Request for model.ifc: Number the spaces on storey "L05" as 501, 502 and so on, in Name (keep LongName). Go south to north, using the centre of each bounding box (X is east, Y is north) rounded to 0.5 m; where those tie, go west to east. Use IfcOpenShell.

First a look at what the model holds.

```python
import ifcopenshell
import ifcopenshell.util.element
import ifcopenshell.util.placement

model = ifcopenshell.open("model.ifc")
print(model.schema)
storey = next(s for s in model.by_type("IfcBuildingStorey") if s.Name == "L05")
spaces = [e for e in ifcopenshell.util.element.get_decomposition(storey) if e.is_a("IfcSpace")]
for e in sorted(spaces, key=lambda e: e.id()):
    origin = ifcopenshell.util.placement.get_local_placement(e.ObjectPlacement)[:3, 3]
    print(e.id(), e.Name, e.LongName, origin.round(2) + 0.0, sep=" | ")
```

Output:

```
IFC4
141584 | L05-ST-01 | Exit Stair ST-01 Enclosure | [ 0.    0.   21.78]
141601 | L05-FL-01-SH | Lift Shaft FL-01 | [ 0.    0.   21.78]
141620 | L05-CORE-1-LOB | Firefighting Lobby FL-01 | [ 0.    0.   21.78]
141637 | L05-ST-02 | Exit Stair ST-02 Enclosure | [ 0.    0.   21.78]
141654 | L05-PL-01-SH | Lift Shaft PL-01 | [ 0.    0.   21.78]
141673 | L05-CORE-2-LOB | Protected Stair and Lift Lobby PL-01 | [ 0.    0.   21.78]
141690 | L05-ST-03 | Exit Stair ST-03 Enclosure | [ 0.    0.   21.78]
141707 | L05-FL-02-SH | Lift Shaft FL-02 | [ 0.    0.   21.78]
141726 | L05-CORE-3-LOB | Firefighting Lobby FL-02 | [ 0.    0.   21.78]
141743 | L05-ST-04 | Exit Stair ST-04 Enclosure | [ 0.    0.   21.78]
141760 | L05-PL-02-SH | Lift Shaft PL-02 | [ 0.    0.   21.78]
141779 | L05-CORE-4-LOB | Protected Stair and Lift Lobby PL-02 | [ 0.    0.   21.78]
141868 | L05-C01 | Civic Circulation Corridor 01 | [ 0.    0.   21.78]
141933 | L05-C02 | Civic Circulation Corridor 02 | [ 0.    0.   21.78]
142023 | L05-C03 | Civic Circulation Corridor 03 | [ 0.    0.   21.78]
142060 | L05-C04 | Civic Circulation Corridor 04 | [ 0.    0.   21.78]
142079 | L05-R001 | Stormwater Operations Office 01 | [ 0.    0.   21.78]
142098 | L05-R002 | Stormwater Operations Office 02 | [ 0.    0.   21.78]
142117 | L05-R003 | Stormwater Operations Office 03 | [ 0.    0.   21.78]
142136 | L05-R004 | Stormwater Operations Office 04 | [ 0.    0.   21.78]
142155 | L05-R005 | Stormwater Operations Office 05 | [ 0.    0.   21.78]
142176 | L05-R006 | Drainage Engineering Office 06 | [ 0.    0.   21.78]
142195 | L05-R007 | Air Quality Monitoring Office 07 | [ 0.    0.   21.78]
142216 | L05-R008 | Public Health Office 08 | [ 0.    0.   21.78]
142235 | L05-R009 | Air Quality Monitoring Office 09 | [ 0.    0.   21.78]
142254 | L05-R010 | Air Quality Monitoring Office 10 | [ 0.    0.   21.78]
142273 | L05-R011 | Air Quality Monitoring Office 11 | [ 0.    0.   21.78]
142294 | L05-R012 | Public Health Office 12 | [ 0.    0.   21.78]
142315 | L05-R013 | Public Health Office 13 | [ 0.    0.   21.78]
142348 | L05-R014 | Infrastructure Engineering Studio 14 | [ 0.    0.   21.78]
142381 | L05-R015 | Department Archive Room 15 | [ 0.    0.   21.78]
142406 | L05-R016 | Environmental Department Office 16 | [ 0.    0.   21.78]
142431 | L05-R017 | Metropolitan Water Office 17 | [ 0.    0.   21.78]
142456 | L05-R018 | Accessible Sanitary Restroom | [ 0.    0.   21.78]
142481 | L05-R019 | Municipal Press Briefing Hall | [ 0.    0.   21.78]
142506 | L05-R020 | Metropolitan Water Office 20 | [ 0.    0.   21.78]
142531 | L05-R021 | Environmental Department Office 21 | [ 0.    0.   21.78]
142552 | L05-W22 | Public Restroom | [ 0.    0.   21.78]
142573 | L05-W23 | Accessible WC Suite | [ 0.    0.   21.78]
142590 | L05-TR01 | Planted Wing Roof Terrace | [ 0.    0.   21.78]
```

```python
import ifcopenshell
import ifcopenshell.geom
import ifcopenshell.util.element
import ifcopenshell.util.shape

model = ifcopenshell.open("model.ifc")
settings = ifcopenshell.geom.settings()
settings.set("use-world-coords", True)


def centre(element):
    shape = ifcopenshell.geom.create_shape(settings, element)
    return ifcopenshell.util.shape.get_bbox_centroid(shape.geometry)


storey = next(s for s in model.by_type("IfcBuildingStorey") if s.Name == "L05")
spaces = [e for e in ifcopenshell.util.element.get_decomposition(storey) if e.is_a("IfcSpace")]

# Insertion points can sit at a corner or the storey origin, so sort by the geometry (in metres).
centres = {e: centre(e) for e in spaces}
spaces.sort(key=lambda e: (round(centres[e][1] / 0.5), centres[e][0]))

for i, e in enumerate(spaces, start=1):
    number = f"5{i:02d}"
    e.Name = number
    print(e.id(), number)

model.write("model_rev.ifc")
```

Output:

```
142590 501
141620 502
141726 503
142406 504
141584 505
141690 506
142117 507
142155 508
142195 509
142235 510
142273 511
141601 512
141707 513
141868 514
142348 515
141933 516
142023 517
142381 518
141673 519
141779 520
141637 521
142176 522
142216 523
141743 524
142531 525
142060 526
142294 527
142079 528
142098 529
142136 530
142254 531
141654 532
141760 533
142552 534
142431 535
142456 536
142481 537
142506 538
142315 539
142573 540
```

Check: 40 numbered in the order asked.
